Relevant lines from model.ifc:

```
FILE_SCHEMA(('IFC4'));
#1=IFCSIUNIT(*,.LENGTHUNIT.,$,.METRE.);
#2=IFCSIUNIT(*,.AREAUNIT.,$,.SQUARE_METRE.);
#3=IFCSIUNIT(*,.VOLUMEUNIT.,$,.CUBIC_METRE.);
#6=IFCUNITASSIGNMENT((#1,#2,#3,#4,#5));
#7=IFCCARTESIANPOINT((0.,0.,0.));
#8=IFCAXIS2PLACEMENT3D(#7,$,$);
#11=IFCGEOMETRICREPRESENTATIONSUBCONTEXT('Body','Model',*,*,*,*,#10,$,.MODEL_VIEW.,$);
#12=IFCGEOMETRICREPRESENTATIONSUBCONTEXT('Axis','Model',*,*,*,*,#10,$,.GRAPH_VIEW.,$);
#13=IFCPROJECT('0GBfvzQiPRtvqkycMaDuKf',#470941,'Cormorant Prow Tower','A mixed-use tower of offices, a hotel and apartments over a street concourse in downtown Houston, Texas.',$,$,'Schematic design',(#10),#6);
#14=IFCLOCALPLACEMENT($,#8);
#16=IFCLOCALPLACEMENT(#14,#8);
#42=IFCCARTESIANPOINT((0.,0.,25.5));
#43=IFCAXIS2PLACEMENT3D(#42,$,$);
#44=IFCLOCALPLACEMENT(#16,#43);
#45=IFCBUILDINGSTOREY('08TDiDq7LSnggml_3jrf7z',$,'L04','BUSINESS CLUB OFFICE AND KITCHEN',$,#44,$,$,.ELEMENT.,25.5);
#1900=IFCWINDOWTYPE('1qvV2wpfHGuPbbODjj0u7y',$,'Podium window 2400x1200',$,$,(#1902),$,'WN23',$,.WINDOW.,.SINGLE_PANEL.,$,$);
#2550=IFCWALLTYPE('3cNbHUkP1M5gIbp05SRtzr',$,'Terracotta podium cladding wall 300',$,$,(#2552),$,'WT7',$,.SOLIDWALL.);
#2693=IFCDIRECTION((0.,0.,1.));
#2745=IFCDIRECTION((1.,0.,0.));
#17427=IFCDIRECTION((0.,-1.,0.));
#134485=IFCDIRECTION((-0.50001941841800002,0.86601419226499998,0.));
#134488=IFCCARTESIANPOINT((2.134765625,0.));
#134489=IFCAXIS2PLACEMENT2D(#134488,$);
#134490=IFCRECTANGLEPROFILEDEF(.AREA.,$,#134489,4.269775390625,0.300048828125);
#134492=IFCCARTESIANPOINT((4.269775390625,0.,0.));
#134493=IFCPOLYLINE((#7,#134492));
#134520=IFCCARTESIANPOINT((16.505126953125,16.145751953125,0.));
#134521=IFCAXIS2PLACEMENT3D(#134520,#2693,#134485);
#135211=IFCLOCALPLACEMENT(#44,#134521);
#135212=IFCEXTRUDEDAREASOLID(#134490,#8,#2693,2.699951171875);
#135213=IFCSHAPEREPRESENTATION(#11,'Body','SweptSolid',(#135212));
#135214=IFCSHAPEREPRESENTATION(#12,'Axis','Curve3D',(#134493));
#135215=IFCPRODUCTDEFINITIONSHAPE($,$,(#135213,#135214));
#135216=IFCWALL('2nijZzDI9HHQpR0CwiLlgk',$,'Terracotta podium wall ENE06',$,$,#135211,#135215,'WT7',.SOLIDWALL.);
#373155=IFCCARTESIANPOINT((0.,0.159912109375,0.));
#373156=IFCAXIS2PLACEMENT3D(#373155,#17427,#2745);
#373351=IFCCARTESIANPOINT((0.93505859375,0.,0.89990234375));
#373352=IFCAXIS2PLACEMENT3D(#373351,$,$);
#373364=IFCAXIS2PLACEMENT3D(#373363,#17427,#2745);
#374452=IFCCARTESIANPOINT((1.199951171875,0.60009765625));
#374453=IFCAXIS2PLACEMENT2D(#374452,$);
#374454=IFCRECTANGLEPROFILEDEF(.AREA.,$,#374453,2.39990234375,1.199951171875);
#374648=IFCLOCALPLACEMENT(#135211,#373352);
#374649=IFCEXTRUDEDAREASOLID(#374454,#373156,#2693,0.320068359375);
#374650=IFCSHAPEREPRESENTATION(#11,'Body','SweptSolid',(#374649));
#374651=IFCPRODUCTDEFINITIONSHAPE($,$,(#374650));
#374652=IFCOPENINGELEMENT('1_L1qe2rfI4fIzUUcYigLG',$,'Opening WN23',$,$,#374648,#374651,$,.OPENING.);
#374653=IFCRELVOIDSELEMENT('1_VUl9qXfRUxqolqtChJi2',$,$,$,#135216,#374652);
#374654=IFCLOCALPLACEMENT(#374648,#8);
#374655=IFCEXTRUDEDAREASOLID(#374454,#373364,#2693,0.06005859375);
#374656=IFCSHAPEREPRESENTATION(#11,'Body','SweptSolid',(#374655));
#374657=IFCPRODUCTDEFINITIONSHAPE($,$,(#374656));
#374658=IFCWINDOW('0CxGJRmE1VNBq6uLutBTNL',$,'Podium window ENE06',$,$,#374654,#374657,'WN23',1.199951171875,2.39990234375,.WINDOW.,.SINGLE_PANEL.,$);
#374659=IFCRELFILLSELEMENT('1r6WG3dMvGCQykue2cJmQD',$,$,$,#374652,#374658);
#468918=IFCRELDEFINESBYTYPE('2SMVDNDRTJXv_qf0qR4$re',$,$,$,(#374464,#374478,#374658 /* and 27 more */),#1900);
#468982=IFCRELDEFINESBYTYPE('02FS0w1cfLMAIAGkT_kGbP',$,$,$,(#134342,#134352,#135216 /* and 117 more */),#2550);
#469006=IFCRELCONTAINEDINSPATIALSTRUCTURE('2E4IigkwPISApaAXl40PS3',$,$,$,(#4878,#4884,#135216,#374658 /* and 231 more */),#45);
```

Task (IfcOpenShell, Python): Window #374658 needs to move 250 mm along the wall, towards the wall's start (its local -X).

```python
import ifcopenshell
import ifcopenshell.api.geometry
import ifcopenshell.util.placement

model = ifcopenshell.open("model.ifc")

window = model.by_guid("0CxGJRmE1VNBq6uLutBTNL")
opening = window.FillsVoids[0].RelatingOpeningElement
wall = opening.VoidsElements[0].RelatingBuildingElement

wall_matrix = ifcopenshell.util.placement.get_local_placement(wall.ObjectPlacement)
shift = wall_matrix[:3, 0] * -0.25
before = ifcopenshell.util.placement.get_local_placement(window.ObjectPlacement)[:3, 3].copy()

# The window is placed relative to its opening, so it follows when the opening moves.
matrix = ifcopenshell.util.placement.get_local_placement(opening.ObjectPlacement)
matrix[:3, 3] += shift
ifcopenshell.api.geometry.edit_object_placement(
    model, product=opening, matrix=matrix, is_si=False, should_transform_children=True
)

after = ifcopenshell.util.placement.get_local_placement(window.ObjectPlacement)[:3, 3]
print("window moved by", (after - before).round(3) + 0.0)

model.write("model_rev.ifc")
```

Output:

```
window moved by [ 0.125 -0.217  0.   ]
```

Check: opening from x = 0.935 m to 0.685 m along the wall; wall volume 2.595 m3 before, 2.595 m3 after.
